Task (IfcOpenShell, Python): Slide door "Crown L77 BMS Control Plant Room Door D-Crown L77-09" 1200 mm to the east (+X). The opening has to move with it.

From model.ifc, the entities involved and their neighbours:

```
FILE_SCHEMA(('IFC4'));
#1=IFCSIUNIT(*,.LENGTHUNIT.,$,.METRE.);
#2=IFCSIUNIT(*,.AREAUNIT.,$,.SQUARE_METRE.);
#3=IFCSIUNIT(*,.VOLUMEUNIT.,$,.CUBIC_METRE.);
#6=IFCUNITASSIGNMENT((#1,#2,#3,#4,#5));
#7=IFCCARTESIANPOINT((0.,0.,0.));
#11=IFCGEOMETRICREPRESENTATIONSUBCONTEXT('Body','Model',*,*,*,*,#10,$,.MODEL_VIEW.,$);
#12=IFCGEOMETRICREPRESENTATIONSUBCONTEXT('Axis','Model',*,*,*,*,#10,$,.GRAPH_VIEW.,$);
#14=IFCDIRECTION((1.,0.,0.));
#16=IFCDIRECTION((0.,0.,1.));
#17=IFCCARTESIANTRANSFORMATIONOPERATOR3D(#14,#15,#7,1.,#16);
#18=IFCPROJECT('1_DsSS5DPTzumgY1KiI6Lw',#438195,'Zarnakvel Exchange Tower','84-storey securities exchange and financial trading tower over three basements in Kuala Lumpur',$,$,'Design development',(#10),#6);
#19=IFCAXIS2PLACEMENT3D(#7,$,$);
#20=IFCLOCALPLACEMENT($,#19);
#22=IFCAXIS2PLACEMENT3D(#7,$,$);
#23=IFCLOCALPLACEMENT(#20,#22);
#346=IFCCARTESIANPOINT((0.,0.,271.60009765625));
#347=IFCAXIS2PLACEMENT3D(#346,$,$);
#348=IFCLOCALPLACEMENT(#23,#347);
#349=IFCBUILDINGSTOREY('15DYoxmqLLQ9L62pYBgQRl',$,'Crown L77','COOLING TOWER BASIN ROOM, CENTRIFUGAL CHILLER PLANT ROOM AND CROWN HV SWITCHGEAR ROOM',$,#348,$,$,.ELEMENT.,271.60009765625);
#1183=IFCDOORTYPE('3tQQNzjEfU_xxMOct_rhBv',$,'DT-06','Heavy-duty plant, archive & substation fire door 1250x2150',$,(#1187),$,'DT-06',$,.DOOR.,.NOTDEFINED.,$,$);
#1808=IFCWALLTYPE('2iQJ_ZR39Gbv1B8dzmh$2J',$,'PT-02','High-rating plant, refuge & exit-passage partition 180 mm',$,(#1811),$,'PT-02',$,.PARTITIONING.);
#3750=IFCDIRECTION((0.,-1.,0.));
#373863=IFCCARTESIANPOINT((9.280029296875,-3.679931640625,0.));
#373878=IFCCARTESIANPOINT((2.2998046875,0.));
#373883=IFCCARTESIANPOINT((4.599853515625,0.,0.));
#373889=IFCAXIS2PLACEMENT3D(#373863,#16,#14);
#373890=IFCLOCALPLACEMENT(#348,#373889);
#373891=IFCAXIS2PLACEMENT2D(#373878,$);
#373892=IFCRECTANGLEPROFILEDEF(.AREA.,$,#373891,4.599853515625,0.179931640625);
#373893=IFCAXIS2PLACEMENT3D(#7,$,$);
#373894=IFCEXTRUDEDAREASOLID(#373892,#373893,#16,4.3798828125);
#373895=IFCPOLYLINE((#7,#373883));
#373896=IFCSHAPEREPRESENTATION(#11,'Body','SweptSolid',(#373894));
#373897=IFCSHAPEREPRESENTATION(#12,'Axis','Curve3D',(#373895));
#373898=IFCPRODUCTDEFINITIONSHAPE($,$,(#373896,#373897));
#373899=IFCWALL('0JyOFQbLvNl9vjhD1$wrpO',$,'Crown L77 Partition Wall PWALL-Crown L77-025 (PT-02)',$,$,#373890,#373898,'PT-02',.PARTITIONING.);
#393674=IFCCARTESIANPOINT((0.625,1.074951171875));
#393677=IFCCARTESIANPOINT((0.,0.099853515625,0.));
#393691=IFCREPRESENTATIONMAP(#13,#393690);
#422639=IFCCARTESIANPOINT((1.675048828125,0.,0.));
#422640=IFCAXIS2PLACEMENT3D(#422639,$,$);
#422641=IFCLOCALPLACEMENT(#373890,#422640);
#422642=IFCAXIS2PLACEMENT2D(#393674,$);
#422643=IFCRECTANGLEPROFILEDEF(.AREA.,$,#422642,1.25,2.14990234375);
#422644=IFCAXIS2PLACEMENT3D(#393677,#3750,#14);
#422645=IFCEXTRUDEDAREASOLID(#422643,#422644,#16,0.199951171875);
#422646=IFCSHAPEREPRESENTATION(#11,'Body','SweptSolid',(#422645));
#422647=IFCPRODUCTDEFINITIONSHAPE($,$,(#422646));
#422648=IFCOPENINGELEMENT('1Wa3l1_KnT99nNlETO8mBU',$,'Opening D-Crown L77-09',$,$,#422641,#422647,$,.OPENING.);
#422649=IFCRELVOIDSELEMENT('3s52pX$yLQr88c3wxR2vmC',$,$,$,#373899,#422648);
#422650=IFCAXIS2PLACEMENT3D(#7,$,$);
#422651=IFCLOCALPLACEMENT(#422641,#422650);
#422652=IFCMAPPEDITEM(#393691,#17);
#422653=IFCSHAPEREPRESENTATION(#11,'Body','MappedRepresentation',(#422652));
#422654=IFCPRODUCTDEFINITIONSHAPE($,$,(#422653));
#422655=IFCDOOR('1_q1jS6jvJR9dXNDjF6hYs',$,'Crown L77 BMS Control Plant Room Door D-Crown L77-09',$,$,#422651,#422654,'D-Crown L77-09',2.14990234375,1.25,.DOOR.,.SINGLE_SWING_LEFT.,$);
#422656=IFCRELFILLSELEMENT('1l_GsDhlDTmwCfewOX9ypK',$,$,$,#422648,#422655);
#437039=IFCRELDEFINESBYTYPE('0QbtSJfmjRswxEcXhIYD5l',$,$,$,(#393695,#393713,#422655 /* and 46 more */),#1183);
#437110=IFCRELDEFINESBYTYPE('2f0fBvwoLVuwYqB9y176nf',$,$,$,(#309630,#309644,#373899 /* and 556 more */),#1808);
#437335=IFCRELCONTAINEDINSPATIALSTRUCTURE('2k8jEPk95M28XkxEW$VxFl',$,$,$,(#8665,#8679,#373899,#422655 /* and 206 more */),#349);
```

```python
import ifcopenshell
import ifcopenshell.api.geometry
import ifcopenshell.util.placement

model = ifcopenshell.open("model.ifc")

door = model.by_guid("1_q1jS6jvJR9dXNDjF6hYs")
opening = door.FillsVoids[0].RelatingOpeningElement
wall = opening.VoidsElements[0].RelatingBuildingElement

wall_matrix = ifcopenshell.util.placement.get_local_placement(wall.ObjectPlacement)
shift = wall_matrix[:3, 0] * 1.2
before = ifcopenshell.util.placement.get_local_placement(door.ObjectPlacement)[:3, 3].copy()

# The door is placed relative to its opening, so it follows when the opening moves.
matrix = ifcopenshell.util.placement.get_local_placement(opening.ObjectPlacement)
matrix[:3, 3] += shift
ifcopenshell.api.geometry.edit_object_placement(
    model, product=opening, matrix=matrix, is_si=False, should_transform_children=True
)

after = ifcopenshell.util.placement.get_local_placement(door.ObjectPlacement)[:3, 3]
print("door moved by", (after - before).round(3) + 0.0)

model.write("model_edited.ifc")
```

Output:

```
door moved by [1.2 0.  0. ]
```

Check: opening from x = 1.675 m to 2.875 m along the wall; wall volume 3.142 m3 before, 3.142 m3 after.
